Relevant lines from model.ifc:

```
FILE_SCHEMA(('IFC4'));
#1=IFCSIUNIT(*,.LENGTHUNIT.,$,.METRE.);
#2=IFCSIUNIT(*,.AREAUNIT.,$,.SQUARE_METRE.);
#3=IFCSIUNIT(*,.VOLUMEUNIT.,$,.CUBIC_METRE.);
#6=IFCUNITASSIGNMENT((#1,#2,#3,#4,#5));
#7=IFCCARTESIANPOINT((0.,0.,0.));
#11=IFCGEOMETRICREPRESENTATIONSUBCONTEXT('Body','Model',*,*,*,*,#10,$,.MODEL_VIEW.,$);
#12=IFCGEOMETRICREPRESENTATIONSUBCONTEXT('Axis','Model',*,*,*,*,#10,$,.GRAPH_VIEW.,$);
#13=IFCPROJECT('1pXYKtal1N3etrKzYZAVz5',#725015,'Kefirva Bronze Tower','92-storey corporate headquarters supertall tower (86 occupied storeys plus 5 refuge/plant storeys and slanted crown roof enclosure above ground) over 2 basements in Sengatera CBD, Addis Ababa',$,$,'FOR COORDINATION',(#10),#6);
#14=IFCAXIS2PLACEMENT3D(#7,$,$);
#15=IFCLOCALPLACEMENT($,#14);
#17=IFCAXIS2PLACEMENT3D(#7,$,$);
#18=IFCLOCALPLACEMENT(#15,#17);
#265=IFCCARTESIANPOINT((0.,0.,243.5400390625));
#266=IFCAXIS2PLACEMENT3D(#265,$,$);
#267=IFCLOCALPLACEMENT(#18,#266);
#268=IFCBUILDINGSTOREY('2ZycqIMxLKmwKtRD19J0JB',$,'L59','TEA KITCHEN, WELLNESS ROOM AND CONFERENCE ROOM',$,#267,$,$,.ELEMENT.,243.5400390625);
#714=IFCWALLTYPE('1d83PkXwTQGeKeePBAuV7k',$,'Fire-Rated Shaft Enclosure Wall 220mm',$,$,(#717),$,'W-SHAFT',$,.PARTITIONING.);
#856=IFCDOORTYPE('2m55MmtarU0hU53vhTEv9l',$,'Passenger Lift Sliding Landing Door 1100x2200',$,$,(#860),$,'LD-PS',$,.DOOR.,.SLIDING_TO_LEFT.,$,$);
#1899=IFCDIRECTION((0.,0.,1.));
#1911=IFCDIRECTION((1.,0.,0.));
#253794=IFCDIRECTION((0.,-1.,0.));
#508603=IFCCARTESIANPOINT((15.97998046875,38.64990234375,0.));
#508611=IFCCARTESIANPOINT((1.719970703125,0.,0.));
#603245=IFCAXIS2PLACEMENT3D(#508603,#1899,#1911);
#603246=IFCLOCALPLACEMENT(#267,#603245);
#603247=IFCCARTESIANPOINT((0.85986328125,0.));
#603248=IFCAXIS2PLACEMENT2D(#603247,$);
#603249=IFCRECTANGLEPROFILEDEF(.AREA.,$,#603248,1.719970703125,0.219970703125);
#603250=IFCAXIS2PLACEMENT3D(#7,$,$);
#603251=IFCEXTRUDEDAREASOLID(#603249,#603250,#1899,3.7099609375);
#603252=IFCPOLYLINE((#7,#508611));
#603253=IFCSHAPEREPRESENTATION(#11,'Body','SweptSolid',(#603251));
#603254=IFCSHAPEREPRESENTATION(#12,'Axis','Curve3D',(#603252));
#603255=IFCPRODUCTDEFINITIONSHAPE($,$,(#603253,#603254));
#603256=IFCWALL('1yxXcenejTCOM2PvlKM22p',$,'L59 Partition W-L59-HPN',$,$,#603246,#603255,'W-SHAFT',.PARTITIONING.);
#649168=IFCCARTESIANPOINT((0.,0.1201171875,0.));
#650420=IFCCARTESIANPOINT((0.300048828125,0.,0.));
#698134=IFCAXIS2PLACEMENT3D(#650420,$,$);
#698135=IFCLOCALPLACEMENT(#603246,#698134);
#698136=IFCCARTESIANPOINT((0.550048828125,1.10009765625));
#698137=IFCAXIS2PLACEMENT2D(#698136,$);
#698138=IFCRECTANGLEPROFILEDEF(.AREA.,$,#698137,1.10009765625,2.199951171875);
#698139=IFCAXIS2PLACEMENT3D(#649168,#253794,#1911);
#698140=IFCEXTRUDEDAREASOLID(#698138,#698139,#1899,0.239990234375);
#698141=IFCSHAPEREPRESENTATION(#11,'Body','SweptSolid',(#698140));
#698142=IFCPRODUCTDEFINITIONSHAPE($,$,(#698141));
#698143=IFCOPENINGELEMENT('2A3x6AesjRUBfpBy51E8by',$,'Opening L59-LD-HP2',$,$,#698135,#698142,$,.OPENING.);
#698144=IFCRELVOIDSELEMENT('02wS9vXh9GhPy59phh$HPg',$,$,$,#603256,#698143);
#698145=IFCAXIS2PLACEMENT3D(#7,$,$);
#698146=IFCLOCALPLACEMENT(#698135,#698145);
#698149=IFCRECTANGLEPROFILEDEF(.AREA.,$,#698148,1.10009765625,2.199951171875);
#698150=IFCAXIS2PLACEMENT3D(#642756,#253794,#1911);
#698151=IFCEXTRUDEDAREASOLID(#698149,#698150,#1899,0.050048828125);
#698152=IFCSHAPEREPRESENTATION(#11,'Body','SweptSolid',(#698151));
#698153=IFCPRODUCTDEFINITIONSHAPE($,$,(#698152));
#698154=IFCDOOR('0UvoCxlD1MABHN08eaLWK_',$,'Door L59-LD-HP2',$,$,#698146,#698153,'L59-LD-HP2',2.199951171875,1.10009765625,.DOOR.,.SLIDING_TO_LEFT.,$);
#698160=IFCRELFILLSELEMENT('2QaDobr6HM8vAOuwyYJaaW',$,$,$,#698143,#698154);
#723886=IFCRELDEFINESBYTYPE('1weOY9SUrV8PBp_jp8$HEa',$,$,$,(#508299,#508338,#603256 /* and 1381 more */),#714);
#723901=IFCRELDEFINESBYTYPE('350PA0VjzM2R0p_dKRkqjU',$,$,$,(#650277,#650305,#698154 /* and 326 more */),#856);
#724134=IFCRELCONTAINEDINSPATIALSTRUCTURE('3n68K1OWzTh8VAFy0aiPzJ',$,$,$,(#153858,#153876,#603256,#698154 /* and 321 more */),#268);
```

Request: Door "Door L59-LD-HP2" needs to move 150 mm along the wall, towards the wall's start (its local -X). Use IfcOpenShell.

```python
import ifcopenshell
import ifcopenshell.api.geometry
import ifcopenshell.util.placement
import ifcopenshell.util.unit

model = ifcopenshell.open("model.ifc")
unit_scale = ifcopenshell.util.unit.calculate_unit_scale(model)

door = model.by_id(698154)
opening = door.FillsVoids[0].RelatingOpeningElement
wall = opening.VoidsElements[0].RelatingBuildingElement

wall_matrix = ifcopenshell.util.placement.get_local_placement(wall.ObjectPlacement)
shift = wall_matrix[:3, 0] * -0.15 / unit_scale
before = ifcopenshell.util.placement.get_local_placement(door.ObjectPlacement)[:3, 3].copy()

# The door is placed relative to its opening, so it follows when the opening moves.
matrix = ifcopenshell.util.placement.get_local_placement(opening.ObjectPlacement)
matrix[:3, 3] += shift
ifcopenshell.api.geometry.edit_object_placement(
    model, product=opening, matrix=matrix, is_si=False, should_transform_children=True
)

after = ifcopenshell.util.placement.get_local_placement(door.ObjectPlacement)[:3, 3]
print("door moved by", (after - before).round(3) + 0.0)

model.write("model_rev.ifc")
```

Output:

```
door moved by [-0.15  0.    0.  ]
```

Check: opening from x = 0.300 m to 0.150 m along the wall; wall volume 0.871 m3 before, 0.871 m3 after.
